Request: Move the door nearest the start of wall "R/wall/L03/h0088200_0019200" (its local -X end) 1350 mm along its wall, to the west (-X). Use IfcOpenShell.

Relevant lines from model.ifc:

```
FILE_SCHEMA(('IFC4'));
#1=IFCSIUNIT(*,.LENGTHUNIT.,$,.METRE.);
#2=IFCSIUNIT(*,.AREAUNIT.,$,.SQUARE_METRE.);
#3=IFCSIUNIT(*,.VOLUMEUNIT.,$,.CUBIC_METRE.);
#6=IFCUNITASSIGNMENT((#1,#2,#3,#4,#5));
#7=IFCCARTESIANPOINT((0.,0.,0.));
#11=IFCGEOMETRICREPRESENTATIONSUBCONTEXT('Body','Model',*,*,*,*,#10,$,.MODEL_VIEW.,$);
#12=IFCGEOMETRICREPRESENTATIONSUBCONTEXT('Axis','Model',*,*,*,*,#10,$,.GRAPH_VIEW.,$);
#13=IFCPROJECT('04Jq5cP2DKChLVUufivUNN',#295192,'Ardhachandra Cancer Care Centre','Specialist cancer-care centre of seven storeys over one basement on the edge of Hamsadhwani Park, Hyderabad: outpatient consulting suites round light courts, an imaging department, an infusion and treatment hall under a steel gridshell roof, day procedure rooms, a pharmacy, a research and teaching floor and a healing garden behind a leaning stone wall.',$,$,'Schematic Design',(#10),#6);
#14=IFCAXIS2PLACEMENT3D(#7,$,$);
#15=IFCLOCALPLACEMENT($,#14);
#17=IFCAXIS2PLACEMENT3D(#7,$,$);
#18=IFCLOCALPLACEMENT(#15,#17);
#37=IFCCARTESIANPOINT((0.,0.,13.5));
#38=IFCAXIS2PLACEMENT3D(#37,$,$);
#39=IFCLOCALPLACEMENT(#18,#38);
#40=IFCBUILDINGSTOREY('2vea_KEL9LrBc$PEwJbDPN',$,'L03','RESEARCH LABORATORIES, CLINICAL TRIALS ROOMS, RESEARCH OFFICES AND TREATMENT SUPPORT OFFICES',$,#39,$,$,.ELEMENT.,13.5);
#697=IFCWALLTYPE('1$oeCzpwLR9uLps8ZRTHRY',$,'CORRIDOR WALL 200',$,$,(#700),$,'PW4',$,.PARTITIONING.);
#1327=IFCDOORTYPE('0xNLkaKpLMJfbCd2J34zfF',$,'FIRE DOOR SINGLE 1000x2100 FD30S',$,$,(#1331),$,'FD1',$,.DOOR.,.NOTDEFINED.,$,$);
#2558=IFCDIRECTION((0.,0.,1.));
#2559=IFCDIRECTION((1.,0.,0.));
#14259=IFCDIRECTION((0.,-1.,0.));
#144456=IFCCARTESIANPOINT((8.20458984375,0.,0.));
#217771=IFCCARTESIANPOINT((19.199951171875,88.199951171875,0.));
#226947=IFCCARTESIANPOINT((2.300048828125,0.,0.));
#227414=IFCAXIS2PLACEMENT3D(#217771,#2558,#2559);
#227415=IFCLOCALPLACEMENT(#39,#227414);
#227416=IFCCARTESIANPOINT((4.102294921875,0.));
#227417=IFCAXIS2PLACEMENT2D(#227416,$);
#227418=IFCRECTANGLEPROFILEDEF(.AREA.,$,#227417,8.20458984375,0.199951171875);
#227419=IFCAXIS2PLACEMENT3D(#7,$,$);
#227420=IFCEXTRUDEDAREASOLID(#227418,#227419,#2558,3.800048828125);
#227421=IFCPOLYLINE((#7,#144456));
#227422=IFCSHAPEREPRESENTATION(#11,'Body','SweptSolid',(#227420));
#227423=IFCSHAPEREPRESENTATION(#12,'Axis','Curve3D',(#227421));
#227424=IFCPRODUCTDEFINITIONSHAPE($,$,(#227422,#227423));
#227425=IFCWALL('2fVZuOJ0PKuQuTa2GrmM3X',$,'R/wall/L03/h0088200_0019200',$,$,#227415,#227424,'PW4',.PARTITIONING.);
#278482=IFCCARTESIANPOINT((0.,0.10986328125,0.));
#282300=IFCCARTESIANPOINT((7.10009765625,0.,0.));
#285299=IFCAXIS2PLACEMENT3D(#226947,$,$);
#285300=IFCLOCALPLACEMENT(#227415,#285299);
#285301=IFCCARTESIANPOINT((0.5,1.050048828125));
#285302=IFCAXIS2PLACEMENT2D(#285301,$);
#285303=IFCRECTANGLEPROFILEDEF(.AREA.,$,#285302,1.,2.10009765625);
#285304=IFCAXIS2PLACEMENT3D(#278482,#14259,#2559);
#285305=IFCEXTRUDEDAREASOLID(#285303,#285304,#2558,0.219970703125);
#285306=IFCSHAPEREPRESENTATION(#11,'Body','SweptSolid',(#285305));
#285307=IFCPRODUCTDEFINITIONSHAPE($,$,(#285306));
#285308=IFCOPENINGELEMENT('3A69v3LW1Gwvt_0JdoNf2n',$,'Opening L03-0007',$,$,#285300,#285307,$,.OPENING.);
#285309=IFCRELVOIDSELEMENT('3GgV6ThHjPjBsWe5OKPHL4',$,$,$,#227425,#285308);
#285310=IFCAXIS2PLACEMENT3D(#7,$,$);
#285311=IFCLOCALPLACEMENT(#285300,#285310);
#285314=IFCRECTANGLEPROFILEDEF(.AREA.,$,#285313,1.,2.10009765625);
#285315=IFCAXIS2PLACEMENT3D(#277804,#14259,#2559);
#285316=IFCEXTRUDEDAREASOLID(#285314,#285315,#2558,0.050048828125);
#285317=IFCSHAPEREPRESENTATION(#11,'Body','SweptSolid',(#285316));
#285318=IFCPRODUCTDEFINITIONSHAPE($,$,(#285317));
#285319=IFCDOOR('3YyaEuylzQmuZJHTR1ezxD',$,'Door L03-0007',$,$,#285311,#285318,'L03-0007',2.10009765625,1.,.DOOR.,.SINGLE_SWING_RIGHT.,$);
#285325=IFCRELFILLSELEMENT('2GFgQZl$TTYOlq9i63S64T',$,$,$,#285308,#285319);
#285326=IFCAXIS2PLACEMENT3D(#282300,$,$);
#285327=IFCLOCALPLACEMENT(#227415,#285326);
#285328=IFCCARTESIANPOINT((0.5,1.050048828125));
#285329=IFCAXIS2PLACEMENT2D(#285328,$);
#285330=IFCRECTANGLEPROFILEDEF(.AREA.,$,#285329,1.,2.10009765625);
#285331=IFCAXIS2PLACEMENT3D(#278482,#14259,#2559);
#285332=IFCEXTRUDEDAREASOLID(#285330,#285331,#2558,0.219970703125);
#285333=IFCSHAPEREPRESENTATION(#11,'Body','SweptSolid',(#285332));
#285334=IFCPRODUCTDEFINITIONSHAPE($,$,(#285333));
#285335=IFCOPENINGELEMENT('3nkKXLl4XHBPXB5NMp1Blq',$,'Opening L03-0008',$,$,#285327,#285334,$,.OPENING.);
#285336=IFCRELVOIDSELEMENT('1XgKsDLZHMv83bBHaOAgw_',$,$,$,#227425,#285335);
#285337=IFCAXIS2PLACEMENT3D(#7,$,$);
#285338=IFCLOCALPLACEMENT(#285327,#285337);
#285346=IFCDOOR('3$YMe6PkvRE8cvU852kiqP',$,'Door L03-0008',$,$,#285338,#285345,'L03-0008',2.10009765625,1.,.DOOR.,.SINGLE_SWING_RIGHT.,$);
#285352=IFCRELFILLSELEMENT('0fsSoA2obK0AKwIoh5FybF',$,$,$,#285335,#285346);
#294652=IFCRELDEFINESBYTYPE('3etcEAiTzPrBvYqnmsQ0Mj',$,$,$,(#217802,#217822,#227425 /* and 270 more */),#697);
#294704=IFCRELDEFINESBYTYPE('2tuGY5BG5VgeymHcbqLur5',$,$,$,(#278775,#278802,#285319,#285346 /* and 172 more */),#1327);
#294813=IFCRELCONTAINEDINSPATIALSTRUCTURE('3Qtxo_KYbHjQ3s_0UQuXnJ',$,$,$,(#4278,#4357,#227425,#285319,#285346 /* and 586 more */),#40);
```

```python
import ifcopenshell
import ifcopenshell.api.geometry
import ifcopenshell.util.placement

model = ifcopenshell.open("model.ifc")

door = model.by_guid("3YyaEuylzQmuZJHTR1ezxD")
opening = door.FillsVoids[0].RelatingOpeningElement
wall = opening.VoidsElements[0].RelatingBuildingElement

wall_matrix = ifcopenshell.util.placement.get_local_placement(wall.ObjectPlacement)
shift = wall_matrix[:3, 0] * -1.35
before = ifcopenshell.util.placement.get_local_placement(door.ObjectPlacement)[:3, 3].copy()

# The door is placed relative to its opening, so it follows when the opening moves.
matrix = ifcopenshell.util.placement.get_local_placement(opening.ObjectPlacement)
matrix[:3, 3] += shift
ifcopenshell.api.geometry.edit_object_placement(
    model, product=opening, matrix=matrix, is_si=False, should_transform_children=True
)

after = ifcopenshell.util.placement.get_local_placement(door.ObjectPlacement)[:3, 3]
print("door moved by", (after - before).round(3) + 0.0)

model.write("model_rev.ifc")
```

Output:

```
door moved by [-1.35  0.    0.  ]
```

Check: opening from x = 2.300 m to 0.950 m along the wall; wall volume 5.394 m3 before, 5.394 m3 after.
